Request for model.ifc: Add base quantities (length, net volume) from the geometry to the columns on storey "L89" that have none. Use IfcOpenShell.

First a look at what the model holds.

```python
import ifcopenshell
import ifcopenshell.util.element
import ifcopenshell.util.unit

model = ifcopenshell.open("model.ifc")
print(model.schema)
for unit_type in ("LENGTHUNIT", "AREAUNIT", "VOLUMEUNIT"):
    print(unit_type, ifcopenshell.util.unit.calculate_unit_scale(model, unit_type))
storey = next(s for s in model.by_type("IfcBuildingStorey") if s.Name == "L89")
columns = [e for e in ifcopenshell.util.element.get_decomposition(storey) if e.is_a("IfcColumn")]
for e in sorted(columns, key=lambda e: e.id()):
    print(e.id(), e.is_a(), e.Name, list(ifcopenshell.util.element.get_psets(e, qtos_only=True)), sep=" | ")
```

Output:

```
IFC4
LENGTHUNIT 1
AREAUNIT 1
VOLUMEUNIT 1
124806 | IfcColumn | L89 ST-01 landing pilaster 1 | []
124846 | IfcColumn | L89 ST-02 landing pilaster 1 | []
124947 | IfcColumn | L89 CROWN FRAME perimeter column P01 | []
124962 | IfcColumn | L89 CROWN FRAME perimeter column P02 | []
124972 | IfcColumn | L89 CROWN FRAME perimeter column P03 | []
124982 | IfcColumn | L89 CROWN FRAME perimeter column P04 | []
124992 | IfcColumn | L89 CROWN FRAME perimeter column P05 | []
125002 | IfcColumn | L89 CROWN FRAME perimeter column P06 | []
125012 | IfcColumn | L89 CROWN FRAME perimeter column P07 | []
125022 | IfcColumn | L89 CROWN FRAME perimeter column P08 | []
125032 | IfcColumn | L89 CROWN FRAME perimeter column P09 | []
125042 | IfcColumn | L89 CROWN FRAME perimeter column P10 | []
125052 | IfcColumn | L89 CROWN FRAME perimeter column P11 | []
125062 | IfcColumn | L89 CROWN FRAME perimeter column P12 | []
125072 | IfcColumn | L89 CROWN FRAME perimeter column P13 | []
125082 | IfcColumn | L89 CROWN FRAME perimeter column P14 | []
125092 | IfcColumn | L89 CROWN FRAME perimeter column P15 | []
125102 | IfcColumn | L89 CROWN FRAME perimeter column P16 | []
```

```python
import ifcopenshell
import ifcopenshell.api.pset
import ifcopenshell.geom
import ifcopenshell.util.element
import ifcopenshell.util.shape
import ifcopenshell.util.unit

model = ifcopenshell.open("model.ifc")
unit_scale = ifcopenshell.util.unit.calculate_unit_scale(model)
volume_scale = ifcopenshell.util.unit.calculate_unit_scale(model, "VOLUMEUNIT")
settings = ifcopenshell.geom.settings()

storey = next(s for s in model.by_type("IfcBuildingStorey") if s.Name == "L89")
columns = [e for e in ifcopenshell.util.element.get_decomposition(storey) if e.is_a("IfcColumn")]

for e in sorted(columns, key=lambda e: e.id()):
    if ifcopenshell.util.element.get_psets(e, qtos_only=True, should_inherit=False):
        continue
    # Geometry comes back in metres, in the element's own axes.
    shape = ifcopenshell.geom.create_shape(settings, e)
    values = {
        "Length": ifcopenshell.util.shape.get_z(shape.geometry) / unit_scale,
        "NetVolume": ifcopenshell.util.shape.get_volume(shape.geometry) / volume_scale,
    }
    qto = ifcopenshell.api.pset.add_qto(model, product=e, name="Qto_ColumnBaseQuantities")
    ifcopenshell.api.pset.edit_qto(model, qto=qto, properties=values)
    print(e.id(), {k: round(v, 3) for k, v in values.items()})

model.write("model_rev.ifc")
```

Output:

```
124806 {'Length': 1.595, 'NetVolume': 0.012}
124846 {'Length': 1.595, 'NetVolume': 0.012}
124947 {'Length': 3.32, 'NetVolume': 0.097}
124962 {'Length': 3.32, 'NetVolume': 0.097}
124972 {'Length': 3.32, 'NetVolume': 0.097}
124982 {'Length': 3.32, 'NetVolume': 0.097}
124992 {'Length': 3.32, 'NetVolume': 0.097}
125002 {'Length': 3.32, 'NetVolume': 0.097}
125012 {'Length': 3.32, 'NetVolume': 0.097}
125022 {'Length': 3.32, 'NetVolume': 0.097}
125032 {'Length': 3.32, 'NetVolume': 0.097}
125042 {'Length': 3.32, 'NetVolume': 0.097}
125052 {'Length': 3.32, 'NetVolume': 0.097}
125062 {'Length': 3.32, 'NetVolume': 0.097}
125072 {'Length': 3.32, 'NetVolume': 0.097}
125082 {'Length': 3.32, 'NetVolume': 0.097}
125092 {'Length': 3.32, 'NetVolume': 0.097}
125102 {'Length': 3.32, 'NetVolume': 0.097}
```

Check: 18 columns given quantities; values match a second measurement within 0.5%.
